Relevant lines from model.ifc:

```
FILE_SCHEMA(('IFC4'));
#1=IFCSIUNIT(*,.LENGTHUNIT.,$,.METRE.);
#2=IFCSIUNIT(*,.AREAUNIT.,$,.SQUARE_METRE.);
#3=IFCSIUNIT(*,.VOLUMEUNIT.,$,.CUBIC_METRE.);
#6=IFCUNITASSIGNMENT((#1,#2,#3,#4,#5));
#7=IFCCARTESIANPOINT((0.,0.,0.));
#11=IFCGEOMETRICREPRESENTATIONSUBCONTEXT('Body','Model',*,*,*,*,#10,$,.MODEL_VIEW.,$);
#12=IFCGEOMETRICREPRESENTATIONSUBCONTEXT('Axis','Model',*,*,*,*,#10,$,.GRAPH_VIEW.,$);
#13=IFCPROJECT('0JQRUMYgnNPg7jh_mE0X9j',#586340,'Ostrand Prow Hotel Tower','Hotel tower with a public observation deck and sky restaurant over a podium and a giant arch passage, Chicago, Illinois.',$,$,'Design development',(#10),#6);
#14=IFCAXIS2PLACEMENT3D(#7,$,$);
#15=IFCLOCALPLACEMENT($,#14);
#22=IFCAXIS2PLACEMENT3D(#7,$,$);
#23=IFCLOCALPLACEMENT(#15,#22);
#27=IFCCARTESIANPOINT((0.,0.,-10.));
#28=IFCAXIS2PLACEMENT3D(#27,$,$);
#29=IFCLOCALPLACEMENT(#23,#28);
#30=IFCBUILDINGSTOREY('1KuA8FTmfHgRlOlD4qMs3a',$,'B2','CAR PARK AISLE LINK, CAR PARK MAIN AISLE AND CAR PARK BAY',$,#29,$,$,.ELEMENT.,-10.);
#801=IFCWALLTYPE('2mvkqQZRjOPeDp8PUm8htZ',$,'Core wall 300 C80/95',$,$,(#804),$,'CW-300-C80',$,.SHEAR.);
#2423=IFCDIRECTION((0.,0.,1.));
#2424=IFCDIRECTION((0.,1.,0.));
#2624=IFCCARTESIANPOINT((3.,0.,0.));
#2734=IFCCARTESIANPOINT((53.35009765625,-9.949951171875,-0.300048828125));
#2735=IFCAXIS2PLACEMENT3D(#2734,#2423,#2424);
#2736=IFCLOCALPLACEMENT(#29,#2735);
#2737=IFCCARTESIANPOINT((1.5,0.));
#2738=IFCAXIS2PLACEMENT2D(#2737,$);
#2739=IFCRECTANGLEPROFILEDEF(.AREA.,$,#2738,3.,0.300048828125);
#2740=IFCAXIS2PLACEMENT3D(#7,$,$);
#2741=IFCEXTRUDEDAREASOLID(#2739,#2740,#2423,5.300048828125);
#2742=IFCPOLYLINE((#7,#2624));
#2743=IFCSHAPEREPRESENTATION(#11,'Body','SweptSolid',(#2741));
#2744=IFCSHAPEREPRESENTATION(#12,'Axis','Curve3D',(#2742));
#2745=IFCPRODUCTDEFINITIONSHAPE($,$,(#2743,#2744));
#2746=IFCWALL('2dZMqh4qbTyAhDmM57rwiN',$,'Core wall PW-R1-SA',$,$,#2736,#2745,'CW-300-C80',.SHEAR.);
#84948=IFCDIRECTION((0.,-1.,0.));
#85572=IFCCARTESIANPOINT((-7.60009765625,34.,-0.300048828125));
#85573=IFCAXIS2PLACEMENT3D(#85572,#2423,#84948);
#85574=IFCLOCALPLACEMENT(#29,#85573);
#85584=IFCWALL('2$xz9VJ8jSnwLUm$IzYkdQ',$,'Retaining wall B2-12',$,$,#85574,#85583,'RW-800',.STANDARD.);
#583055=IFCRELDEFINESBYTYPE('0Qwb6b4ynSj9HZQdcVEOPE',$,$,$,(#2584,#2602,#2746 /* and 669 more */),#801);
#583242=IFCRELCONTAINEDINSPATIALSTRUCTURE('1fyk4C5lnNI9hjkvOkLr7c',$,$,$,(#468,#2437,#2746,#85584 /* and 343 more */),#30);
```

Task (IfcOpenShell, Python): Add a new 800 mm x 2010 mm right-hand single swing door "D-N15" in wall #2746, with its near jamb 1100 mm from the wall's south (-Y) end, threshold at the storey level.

```python
import numpy as np
import ifcopenshell
import ifcopenshell.api.feature
import ifcopenshell.api.geometry
import ifcopenshell.api.root
import ifcopenshell.api.spatial
import ifcopenshell.geom
import ifcopenshell.util.element
import ifcopenshell.util.placement
import ifcopenshell.util.representation
import ifcopenshell.util.shape
import ifcopenshell.util.unit

model = ifcopenshell.open("model.ifc")
unit_scale = ifcopenshell.util.unit.calculate_unit_scale(model)
settings = ifcopenshell.geom.settings()


def volume(element):
    """Net volume in cubic metres, openings subtracted."""
    shape = ifcopenshell.geom.create_shape(settings, element)
    return ifcopenshell.util.shape.get_volume(shape.geometry)


wall = model.by_guid("2dZMqh4qbTyAhDmM57rwiN")
storey = ifcopenshell.util.element.get_container(wall, ifc_class="IfcBuildingStorey")
context = ifcopenshell.util.representation.get_context(model, "Model", "Body", "MODEL_VIEW")
before = volume(wall)

width, height, from_end, sill = 0.8, 2.01, 1.1, 0.0  # metres

# The wall runs along its own X axis, and the end named is its -X end.
wall_shape = ifcopenshell.geom.create_shape(settings, wall)
x, y, z = ifcopenshell.util.shape.get_vertices(wall_shape.geometry).T
start = x.min() + from_end
face, thickness = float(y.min()), float(y.max() - y.min())
wall_matrix = ifcopenshell.util.placement.get_local_placement(wall.ObjectPlacement)
level = ifcopenshell.util.placement.get_local_placement(storey.ObjectPlacement)[2, 3]


def in_wall(x, y):
    """Placement at x, y metres in the wall's axes, at sill height."""
    matrix = wall_matrix.copy()
    matrix[:, 3] = wall_matrix @ np.array([x / unit_scale, y / unit_scale, 0.0, 1.0])
    matrix[2, 3] = level + sill / unit_scale
    return matrix


# Opening: a box that overshoots both wall faces by 50 mm.
opening = ifcopenshell.api.root.create_entity(model, ifc_class="IfcOpeningElement", predefined_type="OPENING")
box = ifcopenshell.api.geometry.add_wall_representation(
    model, context=context, length=width, height=height, thickness=thickness + 0.1
)
ifcopenshell.api.geometry.assign_representation(model, product=opening, representation=box)
ifcopenshell.api.geometry.edit_object_placement(model, product=opening, matrix=in_wall(start, face - 0.05), is_si=False)
ifcopenshell.api.feature.add_feature(model, feature=opening, element=wall)

door = ifcopenshell.api.root.create_entity(model, ifc_class="IfcDoor", name="D-N15", predefined_type="DOOR")
door.OverallWidth, door.OverallHeight = width / unit_scale, height / unit_scale
door.OperationType = "SINGLE_SWING_RIGHT"
body = ifcopenshell.api.geometry.add_door_representation(
    model,
    context=context,
    overall_width=door.OverallWidth,
    overall_height=door.OverallHeight,
    operation_type="SINGLE_SWING_RIGHT",
    lining_properties={"LiningDepth": thickness / unit_scale, "ThresholdDepth": thickness / unit_scale},
)
ifcopenshell.api.geometry.assign_representation(model, product=door, representation=body)
ifcopenshell.api.spatial.assign_container(model, products=[door], relating_structure=storey)
ifcopenshell.api.feature.add_filling(model, opening=opening, element=door)

# The lining spans the wall, so the door starts at the wall face.
ifcopenshell.api.geometry.edit_object_placement(model, product=door, matrix=in_wall(start, face), is_si=False)

after = volume(wall)

print(f"wall volume {before:.3f} -> {after:.3f} m3")

model.write("model_v2.ifc")
```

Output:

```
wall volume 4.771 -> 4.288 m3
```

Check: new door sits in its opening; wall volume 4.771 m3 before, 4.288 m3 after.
